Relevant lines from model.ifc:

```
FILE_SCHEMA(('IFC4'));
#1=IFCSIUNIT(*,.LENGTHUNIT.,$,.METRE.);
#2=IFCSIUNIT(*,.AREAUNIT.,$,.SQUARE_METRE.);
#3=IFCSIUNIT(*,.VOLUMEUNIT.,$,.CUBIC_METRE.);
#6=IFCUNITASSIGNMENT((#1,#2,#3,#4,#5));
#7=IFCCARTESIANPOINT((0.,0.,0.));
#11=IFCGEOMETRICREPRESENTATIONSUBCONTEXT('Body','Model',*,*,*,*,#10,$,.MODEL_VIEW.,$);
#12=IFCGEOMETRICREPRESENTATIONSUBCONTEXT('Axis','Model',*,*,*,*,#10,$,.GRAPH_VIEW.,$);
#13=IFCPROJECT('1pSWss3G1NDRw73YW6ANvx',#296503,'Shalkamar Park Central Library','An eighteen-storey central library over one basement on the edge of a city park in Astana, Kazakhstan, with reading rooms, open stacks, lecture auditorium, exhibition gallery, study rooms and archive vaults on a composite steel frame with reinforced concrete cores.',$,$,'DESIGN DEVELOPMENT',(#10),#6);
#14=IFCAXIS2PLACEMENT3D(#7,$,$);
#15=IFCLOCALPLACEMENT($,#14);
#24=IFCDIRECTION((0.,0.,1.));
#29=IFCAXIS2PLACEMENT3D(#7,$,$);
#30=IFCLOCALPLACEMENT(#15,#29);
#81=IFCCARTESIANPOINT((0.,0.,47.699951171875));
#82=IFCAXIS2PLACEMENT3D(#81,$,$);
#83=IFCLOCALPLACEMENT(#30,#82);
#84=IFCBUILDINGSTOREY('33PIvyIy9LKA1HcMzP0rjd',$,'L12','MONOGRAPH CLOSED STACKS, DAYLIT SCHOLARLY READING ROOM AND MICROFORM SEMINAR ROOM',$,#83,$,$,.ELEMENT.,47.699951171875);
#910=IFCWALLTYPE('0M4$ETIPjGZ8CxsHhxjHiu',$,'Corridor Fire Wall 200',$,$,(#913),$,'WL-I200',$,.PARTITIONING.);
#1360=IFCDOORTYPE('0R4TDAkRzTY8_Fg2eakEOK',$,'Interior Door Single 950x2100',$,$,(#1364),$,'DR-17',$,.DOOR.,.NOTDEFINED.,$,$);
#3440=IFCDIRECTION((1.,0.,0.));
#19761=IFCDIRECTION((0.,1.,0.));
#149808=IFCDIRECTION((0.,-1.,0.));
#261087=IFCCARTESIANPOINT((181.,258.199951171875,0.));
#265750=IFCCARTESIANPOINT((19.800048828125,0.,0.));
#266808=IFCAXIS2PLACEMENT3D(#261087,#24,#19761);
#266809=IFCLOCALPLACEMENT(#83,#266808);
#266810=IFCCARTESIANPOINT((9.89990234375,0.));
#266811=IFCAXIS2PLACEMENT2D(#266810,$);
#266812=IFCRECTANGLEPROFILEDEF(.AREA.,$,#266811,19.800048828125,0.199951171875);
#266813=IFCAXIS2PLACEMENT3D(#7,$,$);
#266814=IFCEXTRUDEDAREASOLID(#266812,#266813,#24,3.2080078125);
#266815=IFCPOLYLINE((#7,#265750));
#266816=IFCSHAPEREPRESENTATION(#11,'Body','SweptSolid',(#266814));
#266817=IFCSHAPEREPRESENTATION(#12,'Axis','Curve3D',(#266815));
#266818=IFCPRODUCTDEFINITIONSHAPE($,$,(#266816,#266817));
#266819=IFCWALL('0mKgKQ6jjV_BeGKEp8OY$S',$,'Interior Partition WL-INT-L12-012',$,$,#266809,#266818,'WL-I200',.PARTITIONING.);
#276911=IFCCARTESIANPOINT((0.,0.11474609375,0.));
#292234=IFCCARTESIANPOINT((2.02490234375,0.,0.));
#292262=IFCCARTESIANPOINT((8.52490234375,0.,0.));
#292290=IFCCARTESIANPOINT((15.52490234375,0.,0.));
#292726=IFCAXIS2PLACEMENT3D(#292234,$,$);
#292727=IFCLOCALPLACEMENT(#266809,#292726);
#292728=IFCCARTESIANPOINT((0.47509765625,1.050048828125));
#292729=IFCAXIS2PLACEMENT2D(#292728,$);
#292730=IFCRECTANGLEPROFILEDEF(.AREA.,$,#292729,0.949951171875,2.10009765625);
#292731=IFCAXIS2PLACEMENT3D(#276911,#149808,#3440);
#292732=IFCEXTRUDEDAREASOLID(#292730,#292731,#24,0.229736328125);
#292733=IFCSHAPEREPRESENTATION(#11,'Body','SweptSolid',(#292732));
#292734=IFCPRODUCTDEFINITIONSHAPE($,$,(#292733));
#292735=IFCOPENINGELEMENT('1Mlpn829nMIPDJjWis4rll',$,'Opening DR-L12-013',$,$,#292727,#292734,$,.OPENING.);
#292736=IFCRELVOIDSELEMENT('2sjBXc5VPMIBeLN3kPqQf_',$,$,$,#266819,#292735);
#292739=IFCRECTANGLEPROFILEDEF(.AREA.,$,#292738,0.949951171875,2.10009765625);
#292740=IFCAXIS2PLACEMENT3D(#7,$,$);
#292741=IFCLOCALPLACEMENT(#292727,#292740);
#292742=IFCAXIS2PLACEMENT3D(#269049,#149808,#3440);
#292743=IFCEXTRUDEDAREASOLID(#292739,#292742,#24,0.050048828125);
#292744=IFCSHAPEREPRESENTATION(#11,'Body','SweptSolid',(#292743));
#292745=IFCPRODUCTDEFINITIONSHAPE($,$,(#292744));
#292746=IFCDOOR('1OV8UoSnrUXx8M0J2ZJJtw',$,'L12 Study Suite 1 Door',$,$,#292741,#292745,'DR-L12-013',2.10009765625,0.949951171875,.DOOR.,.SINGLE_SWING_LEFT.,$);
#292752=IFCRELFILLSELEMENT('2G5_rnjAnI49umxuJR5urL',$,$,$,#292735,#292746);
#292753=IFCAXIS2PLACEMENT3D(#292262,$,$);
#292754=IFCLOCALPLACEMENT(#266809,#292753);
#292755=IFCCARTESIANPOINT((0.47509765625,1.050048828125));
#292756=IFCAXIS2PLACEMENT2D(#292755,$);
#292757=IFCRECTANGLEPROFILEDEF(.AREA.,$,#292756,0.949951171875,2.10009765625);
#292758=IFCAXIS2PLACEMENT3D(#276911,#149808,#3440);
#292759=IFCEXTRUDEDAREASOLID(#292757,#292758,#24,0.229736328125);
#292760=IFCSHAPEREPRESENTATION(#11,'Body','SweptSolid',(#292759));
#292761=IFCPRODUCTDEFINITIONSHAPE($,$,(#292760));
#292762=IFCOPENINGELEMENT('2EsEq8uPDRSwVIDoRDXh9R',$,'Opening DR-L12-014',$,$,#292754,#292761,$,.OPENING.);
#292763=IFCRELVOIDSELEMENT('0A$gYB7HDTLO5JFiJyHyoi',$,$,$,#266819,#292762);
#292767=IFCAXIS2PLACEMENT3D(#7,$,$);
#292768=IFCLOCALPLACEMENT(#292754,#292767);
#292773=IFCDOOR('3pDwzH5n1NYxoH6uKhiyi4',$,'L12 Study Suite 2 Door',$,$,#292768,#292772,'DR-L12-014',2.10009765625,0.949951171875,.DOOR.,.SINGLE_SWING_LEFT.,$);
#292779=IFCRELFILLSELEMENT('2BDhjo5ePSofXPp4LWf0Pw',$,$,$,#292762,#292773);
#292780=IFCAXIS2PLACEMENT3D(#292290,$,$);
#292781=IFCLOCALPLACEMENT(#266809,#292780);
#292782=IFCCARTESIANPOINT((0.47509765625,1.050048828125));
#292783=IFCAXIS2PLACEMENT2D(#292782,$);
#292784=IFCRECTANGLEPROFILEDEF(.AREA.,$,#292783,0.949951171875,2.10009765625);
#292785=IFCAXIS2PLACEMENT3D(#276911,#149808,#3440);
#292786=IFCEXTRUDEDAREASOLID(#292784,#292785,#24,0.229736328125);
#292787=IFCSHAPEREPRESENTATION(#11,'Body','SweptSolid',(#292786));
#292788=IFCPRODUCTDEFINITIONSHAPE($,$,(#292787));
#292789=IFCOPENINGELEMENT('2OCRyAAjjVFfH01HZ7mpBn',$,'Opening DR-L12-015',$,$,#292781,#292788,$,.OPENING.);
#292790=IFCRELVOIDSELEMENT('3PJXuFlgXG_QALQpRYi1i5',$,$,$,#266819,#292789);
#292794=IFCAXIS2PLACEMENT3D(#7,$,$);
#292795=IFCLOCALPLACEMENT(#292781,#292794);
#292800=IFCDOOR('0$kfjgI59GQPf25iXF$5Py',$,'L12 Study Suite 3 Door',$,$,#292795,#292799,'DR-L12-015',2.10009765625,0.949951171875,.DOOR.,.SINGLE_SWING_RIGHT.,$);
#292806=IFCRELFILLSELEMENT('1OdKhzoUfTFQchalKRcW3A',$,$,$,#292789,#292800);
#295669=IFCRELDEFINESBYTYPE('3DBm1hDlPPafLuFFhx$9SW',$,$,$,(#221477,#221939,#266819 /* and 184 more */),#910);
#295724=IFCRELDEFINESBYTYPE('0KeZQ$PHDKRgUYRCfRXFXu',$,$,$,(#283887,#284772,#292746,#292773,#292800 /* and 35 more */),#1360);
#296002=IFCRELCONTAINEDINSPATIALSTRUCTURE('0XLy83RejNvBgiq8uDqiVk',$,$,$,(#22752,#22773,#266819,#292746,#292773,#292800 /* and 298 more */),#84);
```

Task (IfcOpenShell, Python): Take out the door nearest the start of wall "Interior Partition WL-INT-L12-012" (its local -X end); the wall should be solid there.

```python
import ifcopenshell
import ifcopenshell.api.feature
import ifcopenshell.api.root
import ifcopenshell.geom
import ifcopenshell.util.shape

model = ifcopenshell.open("model.ifc")
settings = ifcopenshell.geom.settings()


def volume(element):
    """Net volume in cubic metres, openings subtracted."""
    shape = ifcopenshell.geom.create_shape(settings, element)
    return ifcopenshell.util.shape.get_volume(shape.geometry)


door = model.by_id(292746)
opening = door.FillsVoids[0].RelatingOpeningElement
wall = opening.VoidsElements[0].RelatingBuildingElement
before = volume(wall)

ifcopenshell.api.root.remove_product(model, product=door)
ifcopenshell.api.feature.remove_feature(model, feature=opening)

after = volume(wall)

print(f"wall volume {before:.3f} -> {after:.3f} m3")

model.write("model_updated.ifc")
```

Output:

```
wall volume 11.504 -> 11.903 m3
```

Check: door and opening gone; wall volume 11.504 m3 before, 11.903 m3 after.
